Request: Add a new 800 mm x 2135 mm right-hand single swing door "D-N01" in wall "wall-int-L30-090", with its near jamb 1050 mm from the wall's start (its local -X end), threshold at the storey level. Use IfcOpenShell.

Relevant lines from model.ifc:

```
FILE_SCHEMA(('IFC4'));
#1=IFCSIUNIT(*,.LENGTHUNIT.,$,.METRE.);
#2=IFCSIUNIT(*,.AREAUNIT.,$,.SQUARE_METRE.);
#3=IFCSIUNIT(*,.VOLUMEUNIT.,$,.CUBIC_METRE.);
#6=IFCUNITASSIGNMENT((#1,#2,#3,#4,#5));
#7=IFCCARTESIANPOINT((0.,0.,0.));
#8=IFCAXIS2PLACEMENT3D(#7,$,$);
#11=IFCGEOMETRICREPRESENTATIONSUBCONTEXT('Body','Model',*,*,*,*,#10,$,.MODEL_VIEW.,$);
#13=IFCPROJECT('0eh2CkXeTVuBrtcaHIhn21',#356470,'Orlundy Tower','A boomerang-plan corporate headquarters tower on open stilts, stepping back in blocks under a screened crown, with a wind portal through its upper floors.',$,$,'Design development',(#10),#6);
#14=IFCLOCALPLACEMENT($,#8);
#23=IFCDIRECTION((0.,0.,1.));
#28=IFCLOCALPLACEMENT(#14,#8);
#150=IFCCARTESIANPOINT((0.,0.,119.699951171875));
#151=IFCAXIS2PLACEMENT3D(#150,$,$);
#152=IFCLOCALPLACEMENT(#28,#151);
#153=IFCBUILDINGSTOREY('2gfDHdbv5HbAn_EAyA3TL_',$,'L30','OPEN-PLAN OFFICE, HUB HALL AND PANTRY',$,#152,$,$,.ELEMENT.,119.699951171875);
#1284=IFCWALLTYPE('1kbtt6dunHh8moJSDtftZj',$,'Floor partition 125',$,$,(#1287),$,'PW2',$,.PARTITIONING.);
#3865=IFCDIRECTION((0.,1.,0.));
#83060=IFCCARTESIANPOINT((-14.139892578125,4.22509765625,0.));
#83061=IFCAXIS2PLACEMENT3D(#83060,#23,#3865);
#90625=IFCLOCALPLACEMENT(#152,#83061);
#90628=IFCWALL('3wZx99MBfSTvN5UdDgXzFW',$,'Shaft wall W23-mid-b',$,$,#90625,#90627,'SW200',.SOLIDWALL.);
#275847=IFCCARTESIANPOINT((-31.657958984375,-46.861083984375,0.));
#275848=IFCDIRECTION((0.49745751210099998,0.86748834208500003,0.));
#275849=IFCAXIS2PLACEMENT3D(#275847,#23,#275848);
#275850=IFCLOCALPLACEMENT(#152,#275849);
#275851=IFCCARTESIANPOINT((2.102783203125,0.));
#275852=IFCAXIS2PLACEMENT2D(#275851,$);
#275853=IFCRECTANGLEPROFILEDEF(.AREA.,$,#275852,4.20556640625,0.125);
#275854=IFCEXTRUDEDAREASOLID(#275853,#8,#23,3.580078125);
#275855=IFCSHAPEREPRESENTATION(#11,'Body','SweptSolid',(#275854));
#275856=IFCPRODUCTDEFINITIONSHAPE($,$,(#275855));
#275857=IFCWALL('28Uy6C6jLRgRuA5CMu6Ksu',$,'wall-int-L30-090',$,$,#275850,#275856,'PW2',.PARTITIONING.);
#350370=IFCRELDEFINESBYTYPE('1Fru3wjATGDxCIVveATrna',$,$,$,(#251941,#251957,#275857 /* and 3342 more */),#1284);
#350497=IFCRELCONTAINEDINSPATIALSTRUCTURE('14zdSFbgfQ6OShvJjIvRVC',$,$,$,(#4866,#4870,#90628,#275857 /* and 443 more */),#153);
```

```python
import numpy as np
import ifcopenshell
import ifcopenshell.api.feature
import ifcopenshell.api.geometry
import ifcopenshell.api.root
import ifcopenshell.api.spatial
import ifcopenshell.geom
import ifcopenshell.util.element
import ifcopenshell.util.placement
import ifcopenshell.util.representation
import ifcopenshell.util.shape
import ifcopenshell.util.unit

model = ifcopenshell.open("model.ifc")
unit_scale = ifcopenshell.util.unit.calculate_unit_scale(model)
settings = ifcopenshell.geom.settings()


def volume(element):
    """Net volume in cubic metres, openings subtracted."""
    shape = ifcopenshell.geom.create_shape(settings, element)
    return ifcopenshell.util.shape.get_volume(shape.geometry)


wall = model.by_guid("28Uy6C6jLRgRuA5CMu6Ksu")
storey = ifcopenshell.util.element.get_container(wall, ifc_class="IfcBuildingStorey")
context = ifcopenshell.util.representation.get_context(model, "Model", "Body", "MODEL_VIEW")
before = volume(wall)

width, height, from_end, sill = 0.8, 2.135, 1.05, 0.0  # metres

# The wall runs along its own X axis, and the end named is its -X end.
wall_shape = ifcopenshell.geom.create_shape(settings, wall)
x, y, z = ifcopenshell.util.shape.get_vertices(wall_shape.geometry).T
start = x.min() + from_end
face, thickness = float(y.min()), float(y.max() - y.min())
wall_matrix = ifcopenshell.util.placement.get_local_placement(wall.ObjectPlacement)
level = ifcopenshell.util.placement.get_local_placement(storey.ObjectPlacement)[2, 3]


def in_wall(x, y):
    """Placement at x, y metres in the wall's axes, at sill height."""
    matrix = wall_matrix.copy()
    matrix[:, 3] = wall_matrix @ np.array([x / unit_scale, y / unit_scale, 0.0, 1.0])
    matrix[2, 3] = level + sill / unit_scale
    return matrix


# Opening: a box that overshoots both wall faces by 50 mm.
opening = ifcopenshell.api.root.create_entity(model, ifc_class="IfcOpeningElement", predefined_type="OPENING")
box = ifcopenshell.api.geometry.add_wall_representation(
    model, context=context, length=width, height=height, thickness=thickness + 0.1
)
ifcopenshell.api.geometry.assign_representation(model, product=opening, representation=box)
ifcopenshell.api.geometry.edit_object_placement(model, product=opening, matrix=in_wall(start, face - 0.05), is_si=False)
ifcopenshell.api.feature.add_feature(model, feature=opening, element=wall)

door = ifcopenshell.api.root.create_entity(model, ifc_class="IfcDoor", name="D-N01", predefined_type="DOOR")
door.OverallWidth, door.OverallHeight = width / unit_scale, height / unit_scale
door.OperationType = "SINGLE_SWING_RIGHT"
body = ifcopenshell.api.geometry.add_door_representation(
    model,
    context=context,
    overall_width=door.OverallWidth,
    overall_height=door.OverallHeight,
    operation_type="SINGLE_SWING_RIGHT",
    lining_properties={"LiningDepth": thickness / unit_scale, "ThresholdDepth": thickness / unit_scale},
)
ifcopenshell.api.geometry.assign_representation(model, product=door, representation=body)
ifcopenshell.api.spatial.assign_container(model, products=[door], relating_structure=storey)
ifcopenshell.api.feature.add_filling(model, opening=opening, element=door)

# The lining spans the wall, so the door starts at the wall face.
ifcopenshell.api.geometry.edit_object_placement(model, product=door, matrix=in_wall(start, face), is_si=False)

after = volume(wall)

print(f"wall volume {before:.3f} -> {after:.3f} m3")

model.write("model_updated.ifc")
```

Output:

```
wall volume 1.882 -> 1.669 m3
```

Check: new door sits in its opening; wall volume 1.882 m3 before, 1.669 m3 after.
